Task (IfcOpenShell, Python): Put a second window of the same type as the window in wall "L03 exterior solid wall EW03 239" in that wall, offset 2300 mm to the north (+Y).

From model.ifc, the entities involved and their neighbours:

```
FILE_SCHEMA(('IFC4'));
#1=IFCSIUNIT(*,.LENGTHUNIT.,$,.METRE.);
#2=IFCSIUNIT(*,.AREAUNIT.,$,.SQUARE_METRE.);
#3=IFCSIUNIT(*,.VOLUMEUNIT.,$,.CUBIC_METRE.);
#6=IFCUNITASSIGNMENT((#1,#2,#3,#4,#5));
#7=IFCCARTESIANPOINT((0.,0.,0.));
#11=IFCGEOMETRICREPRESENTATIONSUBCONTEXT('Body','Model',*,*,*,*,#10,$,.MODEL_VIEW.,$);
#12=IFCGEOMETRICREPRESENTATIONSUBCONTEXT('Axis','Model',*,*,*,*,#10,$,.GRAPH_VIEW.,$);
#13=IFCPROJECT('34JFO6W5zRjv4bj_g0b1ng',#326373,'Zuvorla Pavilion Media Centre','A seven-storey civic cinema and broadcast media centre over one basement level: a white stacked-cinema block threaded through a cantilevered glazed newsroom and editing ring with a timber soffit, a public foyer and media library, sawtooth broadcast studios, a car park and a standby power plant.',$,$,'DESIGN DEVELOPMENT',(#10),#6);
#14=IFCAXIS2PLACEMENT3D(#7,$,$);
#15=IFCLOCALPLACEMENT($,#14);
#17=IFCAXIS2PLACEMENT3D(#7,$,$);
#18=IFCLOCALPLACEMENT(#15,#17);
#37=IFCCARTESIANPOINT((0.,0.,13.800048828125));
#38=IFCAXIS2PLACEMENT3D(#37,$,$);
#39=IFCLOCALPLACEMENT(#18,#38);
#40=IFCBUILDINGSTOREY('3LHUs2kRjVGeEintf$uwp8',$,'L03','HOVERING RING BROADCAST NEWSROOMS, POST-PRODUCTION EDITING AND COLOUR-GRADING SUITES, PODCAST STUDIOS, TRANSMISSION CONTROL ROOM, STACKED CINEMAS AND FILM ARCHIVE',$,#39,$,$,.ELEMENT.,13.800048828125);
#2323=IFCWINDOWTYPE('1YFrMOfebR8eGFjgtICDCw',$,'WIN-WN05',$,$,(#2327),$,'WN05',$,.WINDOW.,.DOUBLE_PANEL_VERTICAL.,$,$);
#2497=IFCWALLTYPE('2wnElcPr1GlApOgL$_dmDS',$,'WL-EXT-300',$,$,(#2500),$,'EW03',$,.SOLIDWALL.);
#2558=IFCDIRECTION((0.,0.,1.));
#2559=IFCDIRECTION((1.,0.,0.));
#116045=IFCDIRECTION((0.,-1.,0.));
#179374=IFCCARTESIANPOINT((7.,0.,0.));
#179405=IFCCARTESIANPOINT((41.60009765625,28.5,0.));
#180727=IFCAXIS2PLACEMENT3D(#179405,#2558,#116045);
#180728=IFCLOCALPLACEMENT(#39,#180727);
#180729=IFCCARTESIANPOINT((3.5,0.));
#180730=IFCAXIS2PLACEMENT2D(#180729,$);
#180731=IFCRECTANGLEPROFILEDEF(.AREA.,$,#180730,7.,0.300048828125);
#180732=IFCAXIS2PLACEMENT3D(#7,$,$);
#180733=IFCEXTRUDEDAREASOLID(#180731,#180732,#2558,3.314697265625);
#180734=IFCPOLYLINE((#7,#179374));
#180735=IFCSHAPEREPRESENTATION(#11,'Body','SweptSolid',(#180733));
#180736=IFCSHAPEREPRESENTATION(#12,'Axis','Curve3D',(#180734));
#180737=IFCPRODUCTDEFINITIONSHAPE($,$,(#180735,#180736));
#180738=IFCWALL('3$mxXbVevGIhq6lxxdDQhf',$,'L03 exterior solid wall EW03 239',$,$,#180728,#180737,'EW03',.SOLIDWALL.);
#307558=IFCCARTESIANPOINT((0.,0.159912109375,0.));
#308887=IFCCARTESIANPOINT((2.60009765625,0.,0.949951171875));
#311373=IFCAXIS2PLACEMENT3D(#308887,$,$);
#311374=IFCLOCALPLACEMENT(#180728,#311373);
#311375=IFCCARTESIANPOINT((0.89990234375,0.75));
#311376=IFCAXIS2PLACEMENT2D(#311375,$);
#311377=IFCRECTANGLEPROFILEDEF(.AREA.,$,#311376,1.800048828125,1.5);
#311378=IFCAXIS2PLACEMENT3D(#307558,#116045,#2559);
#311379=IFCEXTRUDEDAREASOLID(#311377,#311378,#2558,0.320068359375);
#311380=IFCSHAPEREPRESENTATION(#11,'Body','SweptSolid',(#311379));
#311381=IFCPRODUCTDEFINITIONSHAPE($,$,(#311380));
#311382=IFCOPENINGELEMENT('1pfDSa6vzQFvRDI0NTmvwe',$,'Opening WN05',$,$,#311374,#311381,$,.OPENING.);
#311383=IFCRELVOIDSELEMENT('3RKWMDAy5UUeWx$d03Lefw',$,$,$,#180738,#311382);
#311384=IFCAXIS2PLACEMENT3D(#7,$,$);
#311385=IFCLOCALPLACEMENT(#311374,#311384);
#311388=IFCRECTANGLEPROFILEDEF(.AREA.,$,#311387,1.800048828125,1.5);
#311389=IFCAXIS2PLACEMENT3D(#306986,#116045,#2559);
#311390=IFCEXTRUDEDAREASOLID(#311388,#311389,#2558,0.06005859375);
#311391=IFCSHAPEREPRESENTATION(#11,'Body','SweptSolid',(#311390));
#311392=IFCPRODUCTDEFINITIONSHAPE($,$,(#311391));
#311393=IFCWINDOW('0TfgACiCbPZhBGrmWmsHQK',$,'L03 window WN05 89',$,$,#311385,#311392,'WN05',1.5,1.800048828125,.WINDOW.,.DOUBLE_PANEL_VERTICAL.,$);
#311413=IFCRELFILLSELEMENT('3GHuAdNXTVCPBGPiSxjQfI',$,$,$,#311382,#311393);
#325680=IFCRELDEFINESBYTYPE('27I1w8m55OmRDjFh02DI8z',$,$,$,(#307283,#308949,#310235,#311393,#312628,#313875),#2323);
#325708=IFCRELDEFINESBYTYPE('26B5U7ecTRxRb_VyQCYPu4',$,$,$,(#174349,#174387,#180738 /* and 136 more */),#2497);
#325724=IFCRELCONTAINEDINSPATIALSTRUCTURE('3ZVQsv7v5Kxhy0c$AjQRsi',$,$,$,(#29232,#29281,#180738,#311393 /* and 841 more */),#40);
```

```python
import ifcopenshell
import ifcopenshell.api.feature
import ifcopenshell.api.geometry
import ifcopenshell.api.root
import ifcopenshell.geom
import ifcopenshell.util.element
import ifcopenshell.util.placement
import ifcopenshell.util.shape
import ifcopenshell.util.unit

model = ifcopenshell.open("model.ifc")
unit_scale = ifcopenshell.util.unit.calculate_unit_scale(model)
settings = ifcopenshell.geom.settings()


def volume(element):
    """Net volume in cubic metres, openings subtracted."""
    shape = ifcopenshell.geom.create_shape(settings, element)
    return ifcopenshell.util.shape.get_volume(shape.geometry)


window = model.by_id(311393)
opening = window.FillsVoids[0].RelatingOpeningElement
wall = opening.VoidsElements[0].RelatingBuildingElement
before = volume(wall)
shift = ifcopenshell.util.placement.get_local_placement(wall.ObjectPlacement)[:3, 0] * -2.3 / unit_scale

# copy_class copies the void relationship, type, container and properties, but no geometry.
new_opening = ifcopenshell.api.root.copy_class(model, product=opening)
new_opening.Representation = ifcopenshell.util.element.copy_deep(
    model, opening.Representation, exclude=["IfcGeometricRepresentationContext", "IfcRepresentationMap"]
)
new_window = ifcopenshell.api.root.copy_class(model, product=window)
new_window.Representation = ifcopenshell.util.element.copy_deep(
    model, window.Representation, exclude=["IfcGeometricRepresentationContext", "IfcRepresentationMap"]
)
new_window.Tag = None
ifcopenshell.api.feature.add_filling(model, opening=new_opening, element=new_window)

for old, new in ((opening, new_opening), (window, new_window)):
    matrix = ifcopenshell.util.placement.get_local_placement(old.ObjectPlacement)
    matrix[:3, 3] += shift
    ifcopenshell.api.geometry.edit_object_placement(model, product=new, matrix=matrix, is_si=False)

after = volume(wall)

print(f"wall volume {before:.3f} -> {after:.3f} m3")

model.write("model_rev.ifc")
```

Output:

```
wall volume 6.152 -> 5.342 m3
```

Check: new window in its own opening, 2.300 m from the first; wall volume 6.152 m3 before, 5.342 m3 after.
